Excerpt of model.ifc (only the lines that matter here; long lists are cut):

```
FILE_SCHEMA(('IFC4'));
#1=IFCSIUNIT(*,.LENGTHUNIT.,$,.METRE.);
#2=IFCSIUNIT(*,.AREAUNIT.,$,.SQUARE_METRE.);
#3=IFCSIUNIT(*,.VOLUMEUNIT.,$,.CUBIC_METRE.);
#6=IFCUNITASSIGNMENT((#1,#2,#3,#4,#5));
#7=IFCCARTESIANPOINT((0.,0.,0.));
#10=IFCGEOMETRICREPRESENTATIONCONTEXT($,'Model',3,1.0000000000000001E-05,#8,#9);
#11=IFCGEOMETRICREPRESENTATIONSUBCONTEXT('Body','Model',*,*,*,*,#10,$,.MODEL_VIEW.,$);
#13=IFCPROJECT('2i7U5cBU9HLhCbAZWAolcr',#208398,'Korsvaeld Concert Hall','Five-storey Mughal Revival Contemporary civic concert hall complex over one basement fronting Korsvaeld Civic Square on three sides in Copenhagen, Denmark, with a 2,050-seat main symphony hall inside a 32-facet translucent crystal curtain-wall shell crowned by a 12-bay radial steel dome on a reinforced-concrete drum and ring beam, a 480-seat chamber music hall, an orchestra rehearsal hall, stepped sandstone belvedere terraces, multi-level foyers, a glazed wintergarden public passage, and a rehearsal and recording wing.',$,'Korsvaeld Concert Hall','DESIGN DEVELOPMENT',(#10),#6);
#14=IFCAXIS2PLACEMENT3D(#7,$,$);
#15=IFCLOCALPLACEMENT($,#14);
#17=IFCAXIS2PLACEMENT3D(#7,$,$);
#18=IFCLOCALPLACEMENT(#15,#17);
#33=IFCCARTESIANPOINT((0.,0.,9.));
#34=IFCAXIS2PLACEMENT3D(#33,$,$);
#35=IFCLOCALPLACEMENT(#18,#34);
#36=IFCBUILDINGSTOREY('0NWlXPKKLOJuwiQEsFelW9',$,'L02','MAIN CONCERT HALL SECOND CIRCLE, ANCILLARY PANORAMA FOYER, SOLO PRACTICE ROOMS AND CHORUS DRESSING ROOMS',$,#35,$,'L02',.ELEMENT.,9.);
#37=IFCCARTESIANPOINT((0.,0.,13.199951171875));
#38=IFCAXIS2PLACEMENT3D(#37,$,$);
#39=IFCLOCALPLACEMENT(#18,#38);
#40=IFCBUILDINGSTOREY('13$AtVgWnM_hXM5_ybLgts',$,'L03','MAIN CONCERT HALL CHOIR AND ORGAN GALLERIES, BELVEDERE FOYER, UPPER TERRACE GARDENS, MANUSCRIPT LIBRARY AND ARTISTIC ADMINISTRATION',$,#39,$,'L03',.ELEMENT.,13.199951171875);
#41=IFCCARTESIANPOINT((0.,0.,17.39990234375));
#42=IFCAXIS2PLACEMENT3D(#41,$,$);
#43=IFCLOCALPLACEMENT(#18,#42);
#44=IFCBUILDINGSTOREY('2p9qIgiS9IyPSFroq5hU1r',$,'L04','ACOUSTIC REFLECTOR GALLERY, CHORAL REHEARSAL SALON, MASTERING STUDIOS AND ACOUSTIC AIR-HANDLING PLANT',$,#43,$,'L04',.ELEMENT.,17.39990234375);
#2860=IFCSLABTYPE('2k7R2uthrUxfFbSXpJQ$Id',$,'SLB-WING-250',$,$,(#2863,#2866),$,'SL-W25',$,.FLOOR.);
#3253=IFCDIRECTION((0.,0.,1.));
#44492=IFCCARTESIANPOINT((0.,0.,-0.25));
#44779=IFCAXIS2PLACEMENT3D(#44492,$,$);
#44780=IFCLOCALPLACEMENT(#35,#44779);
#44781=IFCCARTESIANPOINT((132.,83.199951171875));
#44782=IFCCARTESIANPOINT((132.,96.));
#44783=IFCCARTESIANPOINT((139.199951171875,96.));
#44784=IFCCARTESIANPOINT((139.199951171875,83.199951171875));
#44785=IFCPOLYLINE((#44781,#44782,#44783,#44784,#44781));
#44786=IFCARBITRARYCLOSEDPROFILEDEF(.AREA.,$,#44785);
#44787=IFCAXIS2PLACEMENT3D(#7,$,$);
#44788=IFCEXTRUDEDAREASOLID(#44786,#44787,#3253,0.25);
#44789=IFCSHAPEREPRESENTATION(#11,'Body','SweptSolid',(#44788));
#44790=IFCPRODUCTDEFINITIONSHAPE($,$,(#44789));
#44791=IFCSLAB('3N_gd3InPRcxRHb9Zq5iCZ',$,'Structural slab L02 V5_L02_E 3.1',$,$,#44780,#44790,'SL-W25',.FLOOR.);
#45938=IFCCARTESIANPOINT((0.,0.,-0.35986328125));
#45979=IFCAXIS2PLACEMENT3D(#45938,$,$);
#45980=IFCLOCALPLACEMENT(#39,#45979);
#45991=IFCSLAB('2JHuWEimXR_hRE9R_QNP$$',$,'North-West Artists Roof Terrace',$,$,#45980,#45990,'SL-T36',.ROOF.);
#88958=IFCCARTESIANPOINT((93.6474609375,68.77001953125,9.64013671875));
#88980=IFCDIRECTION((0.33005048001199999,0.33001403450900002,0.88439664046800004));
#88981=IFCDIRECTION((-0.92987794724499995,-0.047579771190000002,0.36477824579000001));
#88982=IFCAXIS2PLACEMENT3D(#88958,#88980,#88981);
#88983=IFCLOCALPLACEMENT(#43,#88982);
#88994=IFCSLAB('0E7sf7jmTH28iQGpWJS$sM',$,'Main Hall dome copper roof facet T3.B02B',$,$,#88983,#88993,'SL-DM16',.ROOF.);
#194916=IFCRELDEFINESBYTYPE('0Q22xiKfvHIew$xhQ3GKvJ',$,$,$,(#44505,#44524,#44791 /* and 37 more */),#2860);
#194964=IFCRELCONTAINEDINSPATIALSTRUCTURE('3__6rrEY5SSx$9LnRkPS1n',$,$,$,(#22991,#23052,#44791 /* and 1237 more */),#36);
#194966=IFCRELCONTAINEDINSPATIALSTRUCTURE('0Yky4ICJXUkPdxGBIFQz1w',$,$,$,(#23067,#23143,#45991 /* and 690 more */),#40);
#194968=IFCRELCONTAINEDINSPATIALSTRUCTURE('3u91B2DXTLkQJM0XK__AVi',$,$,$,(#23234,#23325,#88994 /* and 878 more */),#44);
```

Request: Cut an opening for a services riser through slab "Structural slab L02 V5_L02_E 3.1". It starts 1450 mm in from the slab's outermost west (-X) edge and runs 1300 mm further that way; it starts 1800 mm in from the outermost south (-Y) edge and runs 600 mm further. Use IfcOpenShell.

```python
import numpy as np
import ifcopenshell
import ifcopenshell.api.feature
import ifcopenshell.api.geometry
import ifcopenshell.api.root
import ifcopenshell.geom
import ifcopenshell.util.placement
import ifcopenshell.util.representation
import ifcopenshell.util.shape
import ifcopenshell.util.unit

model = ifcopenshell.open("model.ifc")
unit_scale = ifcopenshell.util.unit.calculate_unit_scale(model)
settings = ifcopenshell.geom.settings()


def volume(element):
    """Net volume in cubic metres, openings subtracted."""
    shape = ifcopenshell.geom.create_shape(settings, element)
    return ifcopenshell.util.shape.get_volume(shape.geometry)


slab = model.by_id(44791)
before = volume(slab)

# Extent in the slab's own axes, in metres. The edges named are its -X and -Y sides.
slab_shape = ifcopenshell.geom.create_shape(settings, slab)
vertices = ifcopenshell.util.shape.get_vertices(slab_shape.geometry)
x_min, y_min, bottom = vertices.min(axis=0)
top = vertices[:, 2].max()

opening = ifcopenshell.api.root.create_entity(model, ifc_class="IfcOpeningElement", name="Services riser opening", predefined_type="OPENING")
context = ifcopenshell.util.representation.get_context(model, "Model", "Body", "MODEL_VIEW")
width, depth = 1.3, 0.6
outline = [(0.0, 0.0), (width, 0.0), (width, depth), (0.0, depth), (0.0, 0.0)]
# Overshoot both faces by 50 mm so the cut is clean.
shape = ifcopenshell.api.geometry.add_slab_representation(
    model, context=context, depth=top - bottom + 0.1, polyline=outline
)
ifcopenshell.api.geometry.assign_representation(model, product=opening, representation=shape)

matrix = ifcopenshell.util.placement.get_local_placement(slab.ObjectPlacement)
matrix[:, 3] = matrix @ np.append(np.array([x_min + 1.45, y_min + 1.8, bottom - 0.05]) / unit_scale, 1.0)
ifcopenshell.api.geometry.edit_object_placement(model, product=opening, matrix=matrix, is_si=False)
ifcopenshell.api.feature.add_feature(model, feature=opening, element=slab)

after = volume(slab)

print(f"slab volume {before:.3f} -> {after:.3f} m3")

model.write("model_updated.ifc")
```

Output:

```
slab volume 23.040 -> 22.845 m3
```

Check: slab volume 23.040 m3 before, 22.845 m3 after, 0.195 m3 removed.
